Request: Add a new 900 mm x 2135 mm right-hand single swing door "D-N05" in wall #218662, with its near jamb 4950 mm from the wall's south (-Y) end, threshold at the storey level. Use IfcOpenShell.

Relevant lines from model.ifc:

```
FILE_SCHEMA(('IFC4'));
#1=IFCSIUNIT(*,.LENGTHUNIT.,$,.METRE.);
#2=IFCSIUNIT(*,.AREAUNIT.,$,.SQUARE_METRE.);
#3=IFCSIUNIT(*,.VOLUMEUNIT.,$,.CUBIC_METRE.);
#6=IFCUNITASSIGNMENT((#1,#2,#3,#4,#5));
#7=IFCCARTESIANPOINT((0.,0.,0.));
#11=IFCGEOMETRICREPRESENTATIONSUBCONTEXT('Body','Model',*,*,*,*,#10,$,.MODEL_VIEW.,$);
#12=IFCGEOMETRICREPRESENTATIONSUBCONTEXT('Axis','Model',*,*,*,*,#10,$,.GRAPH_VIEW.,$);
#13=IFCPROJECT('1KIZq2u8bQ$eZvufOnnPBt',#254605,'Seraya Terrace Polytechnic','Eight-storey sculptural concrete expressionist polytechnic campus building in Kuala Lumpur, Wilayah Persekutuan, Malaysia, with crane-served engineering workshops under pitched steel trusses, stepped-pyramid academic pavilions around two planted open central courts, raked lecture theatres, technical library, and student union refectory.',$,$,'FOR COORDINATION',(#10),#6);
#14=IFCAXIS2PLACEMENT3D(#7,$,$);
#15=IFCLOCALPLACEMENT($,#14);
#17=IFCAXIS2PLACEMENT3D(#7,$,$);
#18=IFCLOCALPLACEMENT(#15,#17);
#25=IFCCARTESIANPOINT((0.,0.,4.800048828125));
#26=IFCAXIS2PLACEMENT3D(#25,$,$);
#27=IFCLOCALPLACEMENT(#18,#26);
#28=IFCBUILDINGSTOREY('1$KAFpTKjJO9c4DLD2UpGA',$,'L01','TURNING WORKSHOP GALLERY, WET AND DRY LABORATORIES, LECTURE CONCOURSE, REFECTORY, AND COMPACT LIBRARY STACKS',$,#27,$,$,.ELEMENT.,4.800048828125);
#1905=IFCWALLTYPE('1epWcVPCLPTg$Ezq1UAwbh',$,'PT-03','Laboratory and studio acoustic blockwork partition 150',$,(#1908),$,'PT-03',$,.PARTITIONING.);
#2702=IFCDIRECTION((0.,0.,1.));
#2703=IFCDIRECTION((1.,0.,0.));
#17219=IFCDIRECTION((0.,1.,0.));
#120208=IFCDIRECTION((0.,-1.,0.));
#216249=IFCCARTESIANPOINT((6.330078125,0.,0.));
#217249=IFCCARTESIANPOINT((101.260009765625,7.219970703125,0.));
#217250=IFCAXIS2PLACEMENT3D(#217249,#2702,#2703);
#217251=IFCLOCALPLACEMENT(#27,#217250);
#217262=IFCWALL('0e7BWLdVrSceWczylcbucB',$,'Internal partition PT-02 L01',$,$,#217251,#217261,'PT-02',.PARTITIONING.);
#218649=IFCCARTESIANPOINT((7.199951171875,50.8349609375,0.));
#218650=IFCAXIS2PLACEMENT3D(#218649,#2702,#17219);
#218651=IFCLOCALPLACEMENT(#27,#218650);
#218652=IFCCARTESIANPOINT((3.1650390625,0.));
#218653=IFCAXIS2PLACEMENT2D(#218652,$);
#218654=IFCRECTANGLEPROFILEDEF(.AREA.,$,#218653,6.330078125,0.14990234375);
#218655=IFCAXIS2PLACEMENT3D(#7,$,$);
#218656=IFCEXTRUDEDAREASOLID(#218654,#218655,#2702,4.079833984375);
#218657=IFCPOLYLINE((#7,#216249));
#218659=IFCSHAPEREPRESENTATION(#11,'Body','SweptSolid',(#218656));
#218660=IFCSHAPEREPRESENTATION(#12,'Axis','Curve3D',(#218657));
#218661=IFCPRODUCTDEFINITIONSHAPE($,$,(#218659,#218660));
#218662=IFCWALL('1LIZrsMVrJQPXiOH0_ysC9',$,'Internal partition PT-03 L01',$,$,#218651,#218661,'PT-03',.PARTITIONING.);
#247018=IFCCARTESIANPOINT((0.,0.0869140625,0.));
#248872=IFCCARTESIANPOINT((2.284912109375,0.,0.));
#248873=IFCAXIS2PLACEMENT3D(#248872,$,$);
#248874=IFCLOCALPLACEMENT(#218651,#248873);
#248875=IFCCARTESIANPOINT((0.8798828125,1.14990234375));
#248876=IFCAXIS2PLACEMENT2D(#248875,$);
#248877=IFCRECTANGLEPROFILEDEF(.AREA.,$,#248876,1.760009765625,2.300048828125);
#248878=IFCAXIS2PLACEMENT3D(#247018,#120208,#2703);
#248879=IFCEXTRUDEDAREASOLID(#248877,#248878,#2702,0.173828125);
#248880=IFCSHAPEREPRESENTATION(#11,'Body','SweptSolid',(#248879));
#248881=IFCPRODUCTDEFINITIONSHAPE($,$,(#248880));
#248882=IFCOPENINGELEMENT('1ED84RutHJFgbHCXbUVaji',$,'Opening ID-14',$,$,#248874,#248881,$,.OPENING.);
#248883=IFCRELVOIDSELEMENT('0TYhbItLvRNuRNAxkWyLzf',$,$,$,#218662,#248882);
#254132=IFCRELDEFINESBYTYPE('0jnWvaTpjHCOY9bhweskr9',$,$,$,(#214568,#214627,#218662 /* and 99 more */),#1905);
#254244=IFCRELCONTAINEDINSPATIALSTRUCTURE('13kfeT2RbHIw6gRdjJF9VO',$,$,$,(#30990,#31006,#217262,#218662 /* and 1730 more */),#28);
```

```python
import numpy as np
import ifcopenshell
import ifcopenshell.api.feature
import ifcopenshell.api.geometry
import ifcopenshell.api.root
import ifcopenshell.api.spatial
import ifcopenshell.geom
import ifcopenshell.util.element
import ifcopenshell.util.placement
import ifcopenshell.util.representation
import ifcopenshell.util.shape
import ifcopenshell.util.unit

model = ifcopenshell.open("model.ifc")
unit_scale = ifcopenshell.util.unit.calculate_unit_scale(model)
settings = ifcopenshell.geom.settings()


def volume(element):
    """Net volume in cubic metres, openings subtracted."""
    shape = ifcopenshell.geom.create_shape(settings, element)
    return ifcopenshell.util.shape.get_volume(shape.geometry)


wall = model.by_guid("1LIZrsMVrJQPXiOH0_ysC9")
storey = ifcopenshell.util.element.get_container(wall, ifc_class="IfcBuildingStorey")
context = ifcopenshell.util.representation.get_context(model, "Model", "Body", "MODEL_VIEW")
before = volume(wall)

width, height, from_end, sill = 0.9, 2.135, 4.95, 0.0  # metres

# The wall runs along its own X axis, and the end named is its -X end.
wall_shape = ifcopenshell.geom.create_shape(settings, wall)
x, y, z = ifcopenshell.util.shape.get_vertices(wall_shape.geometry).T
start = x.min() + from_end
face, thickness = float(y.min()), float(y.max() - y.min())
wall_matrix = ifcopenshell.util.placement.get_local_placement(wall.ObjectPlacement)
level = ifcopenshell.util.placement.get_local_placement(storey.ObjectPlacement)[2, 3]


def in_wall(x, y):
    """Placement at x, y metres in the wall's axes, at sill height."""
    matrix = wall_matrix.copy()
    matrix[:, 3] = wall_matrix @ np.array([x / unit_scale, y / unit_scale, 0.0, 1.0])
    matrix[2, 3] = level + sill / unit_scale
    return matrix


# Opening: a box that overshoots both wall faces by 50 mm.
opening = ifcopenshell.api.root.create_entity(model, ifc_class="IfcOpeningElement", predefined_type="OPENING")
box = ifcopenshell.api.geometry.add_wall_representation(
    model, context=context, length=width, height=height, thickness=thickness + 0.1
)
ifcopenshell.api.geometry.assign_representation(model, product=opening, representation=box)
ifcopenshell.api.geometry.edit_object_placement(model, product=opening, matrix=in_wall(start, face - 0.05), is_si=False)
ifcopenshell.api.feature.add_feature(model, feature=opening, element=wall)

door = ifcopenshell.api.root.create_entity(model, ifc_class="IfcDoor", name="D-N05", predefined_type="DOOR")
door.OverallWidth, door.OverallHeight = width / unit_scale, height / unit_scale
door.OperationType = "SINGLE_SWING_RIGHT"
body = ifcopenshell.api.geometry.add_door_representation(
    model,
    context=context,
    overall_width=door.OverallWidth,
    overall_height=door.OverallHeight,
    operation_type="SINGLE_SWING_RIGHT",
    lining_properties={"LiningDepth": thickness / unit_scale, "ThresholdDepth": thickness / unit_scale},
)
ifcopenshell.api.geometry.assign_representation(model, product=door, representation=body)
ifcopenshell.api.spatial.assign_container(model, products=[door], relating_structure=storey)
ifcopenshell.api.feature.add_filling(model, opening=opening, element=door)

# The lining spans the wall, so the door starts at the wall face.
ifcopenshell.api.geometry.edit_object_placement(model, product=door, matrix=in_wall(start, face), is_si=False)

after = volume(wall)

print(f"wall volume {before:.3f} -> {after:.3f} m3")

model.write("model_v2.ifc")
```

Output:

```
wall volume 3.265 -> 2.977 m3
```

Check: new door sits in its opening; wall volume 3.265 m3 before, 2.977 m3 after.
